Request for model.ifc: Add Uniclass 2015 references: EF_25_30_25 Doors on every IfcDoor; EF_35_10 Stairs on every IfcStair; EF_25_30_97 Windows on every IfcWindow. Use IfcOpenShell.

First a look at what the model holds.

```python
import ifcopenshell

model = ifcopenshell.open("model.ifc")
print(model.schema)
print("classifications:", [c.Name for c in model.by_type("IfcClassification")])
for ifc_class in ("IfcDoor", "IfcRoof", "IfcStair", "IfcWall", "IfcWindow"):
    print(ifc_class, len(model.by_type(ifc_class)))
```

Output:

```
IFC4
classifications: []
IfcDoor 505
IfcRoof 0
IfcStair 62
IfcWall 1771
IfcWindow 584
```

```python
import ifcopenshell
import ifcopenshell.api.classification

model = ifcopenshell.open("model.ifc")

system = ifcopenshell.api.classification.add_classification(model, classification="Uniclass 2015")

codes = {
    "IfcDoor": ("EF_25_30_25", "Doors"),
    "IfcStair": ("EF_35_10", "Stairs"),
    "IfcWindow": ("EF_25_30_97", "Windows"),
}
for ifc_class, (code, name) in codes.items():
    products = model.by_type(ifc_class)
    ifcopenshell.api.classification.add_reference(
        model, products=products, classification=system, identification=code, name=name
    )
    print(code, len(products))

model.write("model-out.ifc")
```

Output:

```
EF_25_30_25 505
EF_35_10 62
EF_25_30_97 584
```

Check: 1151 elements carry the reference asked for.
